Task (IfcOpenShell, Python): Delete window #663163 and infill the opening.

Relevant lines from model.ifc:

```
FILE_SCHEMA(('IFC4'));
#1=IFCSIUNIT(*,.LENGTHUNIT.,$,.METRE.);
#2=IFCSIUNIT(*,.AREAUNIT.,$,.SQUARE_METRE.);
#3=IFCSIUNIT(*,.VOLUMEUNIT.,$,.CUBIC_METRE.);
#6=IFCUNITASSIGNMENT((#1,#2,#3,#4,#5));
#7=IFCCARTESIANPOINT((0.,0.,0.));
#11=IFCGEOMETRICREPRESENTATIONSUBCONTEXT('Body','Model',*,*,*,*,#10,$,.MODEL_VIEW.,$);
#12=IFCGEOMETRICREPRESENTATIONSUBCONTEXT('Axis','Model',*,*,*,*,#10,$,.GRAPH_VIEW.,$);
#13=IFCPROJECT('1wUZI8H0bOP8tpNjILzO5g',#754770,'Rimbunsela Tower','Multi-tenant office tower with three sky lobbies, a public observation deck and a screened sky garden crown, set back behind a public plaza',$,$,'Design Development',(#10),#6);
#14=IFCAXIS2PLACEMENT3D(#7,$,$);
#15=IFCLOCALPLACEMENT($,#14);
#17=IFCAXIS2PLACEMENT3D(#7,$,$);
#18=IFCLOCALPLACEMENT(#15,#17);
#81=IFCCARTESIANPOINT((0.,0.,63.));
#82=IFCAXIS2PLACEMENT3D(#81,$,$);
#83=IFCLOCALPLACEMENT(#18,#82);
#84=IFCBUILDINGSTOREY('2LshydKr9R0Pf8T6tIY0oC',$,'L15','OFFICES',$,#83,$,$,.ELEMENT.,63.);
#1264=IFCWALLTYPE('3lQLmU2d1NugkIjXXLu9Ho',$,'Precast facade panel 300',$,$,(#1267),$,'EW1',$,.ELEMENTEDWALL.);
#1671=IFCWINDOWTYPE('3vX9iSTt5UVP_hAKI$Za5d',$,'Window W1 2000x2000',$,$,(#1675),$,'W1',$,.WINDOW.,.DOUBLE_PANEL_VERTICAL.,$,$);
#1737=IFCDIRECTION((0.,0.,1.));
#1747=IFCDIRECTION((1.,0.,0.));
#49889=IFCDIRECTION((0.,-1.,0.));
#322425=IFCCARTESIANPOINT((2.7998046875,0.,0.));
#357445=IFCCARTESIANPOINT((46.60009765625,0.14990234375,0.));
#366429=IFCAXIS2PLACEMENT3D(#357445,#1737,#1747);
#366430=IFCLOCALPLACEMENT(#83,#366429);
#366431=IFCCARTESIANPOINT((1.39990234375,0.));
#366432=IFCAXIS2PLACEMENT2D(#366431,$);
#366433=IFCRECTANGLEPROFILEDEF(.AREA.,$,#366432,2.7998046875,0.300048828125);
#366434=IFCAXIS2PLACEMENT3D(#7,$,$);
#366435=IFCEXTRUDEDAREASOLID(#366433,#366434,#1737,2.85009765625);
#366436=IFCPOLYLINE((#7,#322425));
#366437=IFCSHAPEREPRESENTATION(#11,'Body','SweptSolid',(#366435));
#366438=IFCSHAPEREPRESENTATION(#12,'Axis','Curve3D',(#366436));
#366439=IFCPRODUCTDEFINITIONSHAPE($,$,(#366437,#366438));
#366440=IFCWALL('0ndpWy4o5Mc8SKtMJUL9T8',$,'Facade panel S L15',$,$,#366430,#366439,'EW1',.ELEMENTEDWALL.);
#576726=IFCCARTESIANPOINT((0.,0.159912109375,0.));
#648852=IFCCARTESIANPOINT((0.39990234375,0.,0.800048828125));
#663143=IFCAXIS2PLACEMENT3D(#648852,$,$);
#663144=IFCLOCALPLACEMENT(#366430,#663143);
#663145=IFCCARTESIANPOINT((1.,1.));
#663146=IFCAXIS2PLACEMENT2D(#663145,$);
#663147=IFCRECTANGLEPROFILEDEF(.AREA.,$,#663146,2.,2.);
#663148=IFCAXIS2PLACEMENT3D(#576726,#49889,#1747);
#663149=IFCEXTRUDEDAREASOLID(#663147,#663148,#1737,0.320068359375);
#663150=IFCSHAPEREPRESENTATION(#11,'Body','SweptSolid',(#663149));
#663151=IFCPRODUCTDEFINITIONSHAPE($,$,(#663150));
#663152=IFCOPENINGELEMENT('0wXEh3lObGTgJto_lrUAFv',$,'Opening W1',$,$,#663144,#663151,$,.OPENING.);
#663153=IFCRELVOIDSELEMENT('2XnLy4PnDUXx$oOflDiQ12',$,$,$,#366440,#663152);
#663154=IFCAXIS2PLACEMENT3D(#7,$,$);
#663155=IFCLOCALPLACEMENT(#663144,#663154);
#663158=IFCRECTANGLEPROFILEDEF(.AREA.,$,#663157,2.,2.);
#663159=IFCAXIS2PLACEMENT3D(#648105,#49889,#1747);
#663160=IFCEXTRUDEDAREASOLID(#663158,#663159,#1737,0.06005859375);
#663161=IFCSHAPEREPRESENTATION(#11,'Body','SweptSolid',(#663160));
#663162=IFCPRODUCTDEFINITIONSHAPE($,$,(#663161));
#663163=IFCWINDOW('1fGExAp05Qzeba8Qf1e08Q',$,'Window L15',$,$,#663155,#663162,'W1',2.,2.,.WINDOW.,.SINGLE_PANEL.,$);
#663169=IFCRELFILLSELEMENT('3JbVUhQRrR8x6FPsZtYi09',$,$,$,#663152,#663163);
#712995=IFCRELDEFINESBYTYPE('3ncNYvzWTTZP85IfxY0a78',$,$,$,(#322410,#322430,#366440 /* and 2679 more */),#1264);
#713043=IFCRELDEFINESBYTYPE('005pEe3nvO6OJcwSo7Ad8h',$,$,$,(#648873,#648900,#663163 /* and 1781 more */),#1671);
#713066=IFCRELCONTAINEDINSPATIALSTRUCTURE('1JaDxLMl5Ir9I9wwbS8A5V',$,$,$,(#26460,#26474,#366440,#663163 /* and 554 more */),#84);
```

```python
import ifcopenshell
import ifcopenshell.api.feature
import ifcopenshell.api.root
import ifcopenshell.geom
import ifcopenshell.util.shape

model = ifcopenshell.open("model.ifc")
settings = ifcopenshell.geom.settings()


def volume(element):
    """Net volume in cubic metres, openings subtracted."""
    shape = ifcopenshell.geom.create_shape(settings, element)
    return ifcopenshell.util.shape.get_volume(shape.geometry)


window = model.by_guid("1fGExAp05Qzeba8Qf1e08Q")
opening = window.FillsVoids[0].RelatingOpeningElement
wall = opening.VoidsElements[0].RelatingBuildingElement
before = volume(wall)

ifcopenshell.api.root.remove_product(model, product=window)
ifcopenshell.api.feature.remove_feature(model, feature=opening)

after = volume(wall)

print(f"wall volume {before:.3f} -> {after:.3f} m3")

model.write("model_updated.ifc")
```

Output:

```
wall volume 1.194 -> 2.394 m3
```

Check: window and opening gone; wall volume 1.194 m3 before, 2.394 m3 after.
